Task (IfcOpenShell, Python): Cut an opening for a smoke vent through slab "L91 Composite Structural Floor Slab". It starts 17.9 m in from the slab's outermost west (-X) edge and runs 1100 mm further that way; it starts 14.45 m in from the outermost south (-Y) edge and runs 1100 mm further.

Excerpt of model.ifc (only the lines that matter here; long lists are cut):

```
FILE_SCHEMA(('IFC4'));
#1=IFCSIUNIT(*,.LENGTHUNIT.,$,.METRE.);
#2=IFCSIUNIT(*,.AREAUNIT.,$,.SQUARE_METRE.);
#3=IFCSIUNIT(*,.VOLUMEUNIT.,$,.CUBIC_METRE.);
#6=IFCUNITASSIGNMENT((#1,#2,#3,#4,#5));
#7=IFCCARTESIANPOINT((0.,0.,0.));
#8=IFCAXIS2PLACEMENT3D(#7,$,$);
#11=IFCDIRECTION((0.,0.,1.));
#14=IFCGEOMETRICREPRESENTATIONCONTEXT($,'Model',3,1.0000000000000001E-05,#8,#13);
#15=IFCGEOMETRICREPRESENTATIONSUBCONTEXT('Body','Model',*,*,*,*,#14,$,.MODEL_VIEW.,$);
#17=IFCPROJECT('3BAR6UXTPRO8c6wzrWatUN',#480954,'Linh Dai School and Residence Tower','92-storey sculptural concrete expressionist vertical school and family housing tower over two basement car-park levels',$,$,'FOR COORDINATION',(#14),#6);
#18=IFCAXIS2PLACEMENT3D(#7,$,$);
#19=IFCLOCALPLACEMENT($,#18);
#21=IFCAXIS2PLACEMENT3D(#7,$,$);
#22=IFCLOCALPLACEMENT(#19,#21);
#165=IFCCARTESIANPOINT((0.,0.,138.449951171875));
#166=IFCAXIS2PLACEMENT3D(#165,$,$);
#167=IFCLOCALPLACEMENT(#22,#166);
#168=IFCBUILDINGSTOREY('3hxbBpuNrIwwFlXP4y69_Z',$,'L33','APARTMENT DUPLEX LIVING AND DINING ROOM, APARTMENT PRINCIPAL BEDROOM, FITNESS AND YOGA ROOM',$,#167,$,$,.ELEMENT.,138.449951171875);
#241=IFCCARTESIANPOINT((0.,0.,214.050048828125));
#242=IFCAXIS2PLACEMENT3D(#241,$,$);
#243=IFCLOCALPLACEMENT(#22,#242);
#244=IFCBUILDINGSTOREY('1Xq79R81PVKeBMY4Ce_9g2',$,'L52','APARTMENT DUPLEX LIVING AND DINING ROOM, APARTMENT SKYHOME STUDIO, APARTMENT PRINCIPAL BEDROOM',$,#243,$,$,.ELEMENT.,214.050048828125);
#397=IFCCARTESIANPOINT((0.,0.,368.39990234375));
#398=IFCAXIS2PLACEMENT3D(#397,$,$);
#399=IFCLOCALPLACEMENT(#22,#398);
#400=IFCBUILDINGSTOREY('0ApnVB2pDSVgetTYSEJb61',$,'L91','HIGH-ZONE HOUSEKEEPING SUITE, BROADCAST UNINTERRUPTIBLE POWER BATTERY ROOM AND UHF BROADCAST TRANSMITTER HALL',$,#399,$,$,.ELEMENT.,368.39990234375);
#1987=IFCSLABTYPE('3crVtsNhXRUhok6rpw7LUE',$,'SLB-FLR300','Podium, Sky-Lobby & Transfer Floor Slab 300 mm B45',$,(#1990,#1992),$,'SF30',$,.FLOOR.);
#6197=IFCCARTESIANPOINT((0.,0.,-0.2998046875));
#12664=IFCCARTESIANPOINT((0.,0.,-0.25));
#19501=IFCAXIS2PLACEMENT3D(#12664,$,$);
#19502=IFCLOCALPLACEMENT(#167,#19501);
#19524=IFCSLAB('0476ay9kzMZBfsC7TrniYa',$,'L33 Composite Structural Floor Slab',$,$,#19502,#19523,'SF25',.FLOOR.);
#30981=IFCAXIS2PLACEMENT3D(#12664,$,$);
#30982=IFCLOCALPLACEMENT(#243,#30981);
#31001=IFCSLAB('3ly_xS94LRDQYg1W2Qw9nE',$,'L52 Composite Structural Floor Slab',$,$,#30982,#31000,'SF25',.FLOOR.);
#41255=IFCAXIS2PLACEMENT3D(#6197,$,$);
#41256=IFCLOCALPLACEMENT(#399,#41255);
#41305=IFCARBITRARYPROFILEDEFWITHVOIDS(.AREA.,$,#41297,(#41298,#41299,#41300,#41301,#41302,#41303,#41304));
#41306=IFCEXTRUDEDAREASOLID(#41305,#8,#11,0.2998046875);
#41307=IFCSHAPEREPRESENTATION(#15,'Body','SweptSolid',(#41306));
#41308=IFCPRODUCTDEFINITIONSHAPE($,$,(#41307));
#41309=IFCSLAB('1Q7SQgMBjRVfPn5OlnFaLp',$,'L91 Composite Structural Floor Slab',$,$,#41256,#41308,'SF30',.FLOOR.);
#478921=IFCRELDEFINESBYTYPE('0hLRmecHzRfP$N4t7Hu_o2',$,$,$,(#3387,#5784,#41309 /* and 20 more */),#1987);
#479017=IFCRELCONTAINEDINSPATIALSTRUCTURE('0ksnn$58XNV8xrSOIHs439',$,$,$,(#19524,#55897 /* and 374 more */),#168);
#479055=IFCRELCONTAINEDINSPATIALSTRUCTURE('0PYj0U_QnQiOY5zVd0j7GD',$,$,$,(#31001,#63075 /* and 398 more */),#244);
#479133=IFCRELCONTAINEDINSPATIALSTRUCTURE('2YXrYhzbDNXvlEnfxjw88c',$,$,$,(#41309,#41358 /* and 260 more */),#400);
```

```python
import numpy as np
import ifcopenshell
import ifcopenshell.api.feature
import ifcopenshell.api.geometry
import ifcopenshell.api.root
import ifcopenshell.geom
import ifcopenshell.util.placement
import ifcopenshell.util.representation
import ifcopenshell.util.shape
import ifcopenshell.util.unit

model = ifcopenshell.open("model.ifc")
unit_scale = ifcopenshell.util.unit.calculate_unit_scale(model)
settings = ifcopenshell.geom.settings()


def volume(element):
    """Net volume in cubic metres, openings subtracted."""
    shape = ifcopenshell.geom.create_shape(settings, element)
    return ifcopenshell.util.shape.get_volume(shape.geometry)


slab = model.by_id(41309)
before = volume(slab)

# Extent in the slab's own axes, in metres. The edges named are its -X and -Y sides.
slab_shape = ifcopenshell.geom.create_shape(settings, slab)
vertices = ifcopenshell.util.shape.get_vertices(slab_shape.geometry)
x_min, y_min, bottom = vertices.min(axis=0)
top = vertices[:, 2].max()

opening = ifcopenshell.api.root.create_entity(model, ifc_class="IfcOpeningElement", name="Smoke vent opening", predefined_type="OPENING")
context = ifcopenshell.util.representation.get_context(model, "Model", "Body", "MODEL_VIEW")
width, depth = 1.1, 1.1
outline = [(0.0, 0.0), (width, 0.0), (width, depth), (0.0, depth), (0.0, 0.0)]
# Overshoot both faces by 50 mm so the cut is clean.
shape = ifcopenshell.api.geometry.add_slab_representation(
    model, context=context, depth=top - bottom + 0.1, polyline=outline
)
ifcopenshell.api.geometry.assign_representation(model, product=opening, representation=shape)

matrix = ifcopenshell.util.placement.get_local_placement(slab.ObjectPlacement)
matrix[:, 3] = matrix @ np.append(np.array([x_min + 17.9, y_min + 14.45, bottom - 0.05]) / unit_scale, 1.0)
ifcopenshell.api.geometry.edit_object_placement(model, product=opening, matrix=matrix, is_si=False)
ifcopenshell.api.feature.add_feature(model, feature=opening, element=slab)

after = volume(slab)

print(f"slab volume {before:.3f} -> {after:.3f} m3")

model.write("model_updated.ifc")
```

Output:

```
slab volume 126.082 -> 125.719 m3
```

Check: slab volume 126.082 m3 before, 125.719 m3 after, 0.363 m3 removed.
